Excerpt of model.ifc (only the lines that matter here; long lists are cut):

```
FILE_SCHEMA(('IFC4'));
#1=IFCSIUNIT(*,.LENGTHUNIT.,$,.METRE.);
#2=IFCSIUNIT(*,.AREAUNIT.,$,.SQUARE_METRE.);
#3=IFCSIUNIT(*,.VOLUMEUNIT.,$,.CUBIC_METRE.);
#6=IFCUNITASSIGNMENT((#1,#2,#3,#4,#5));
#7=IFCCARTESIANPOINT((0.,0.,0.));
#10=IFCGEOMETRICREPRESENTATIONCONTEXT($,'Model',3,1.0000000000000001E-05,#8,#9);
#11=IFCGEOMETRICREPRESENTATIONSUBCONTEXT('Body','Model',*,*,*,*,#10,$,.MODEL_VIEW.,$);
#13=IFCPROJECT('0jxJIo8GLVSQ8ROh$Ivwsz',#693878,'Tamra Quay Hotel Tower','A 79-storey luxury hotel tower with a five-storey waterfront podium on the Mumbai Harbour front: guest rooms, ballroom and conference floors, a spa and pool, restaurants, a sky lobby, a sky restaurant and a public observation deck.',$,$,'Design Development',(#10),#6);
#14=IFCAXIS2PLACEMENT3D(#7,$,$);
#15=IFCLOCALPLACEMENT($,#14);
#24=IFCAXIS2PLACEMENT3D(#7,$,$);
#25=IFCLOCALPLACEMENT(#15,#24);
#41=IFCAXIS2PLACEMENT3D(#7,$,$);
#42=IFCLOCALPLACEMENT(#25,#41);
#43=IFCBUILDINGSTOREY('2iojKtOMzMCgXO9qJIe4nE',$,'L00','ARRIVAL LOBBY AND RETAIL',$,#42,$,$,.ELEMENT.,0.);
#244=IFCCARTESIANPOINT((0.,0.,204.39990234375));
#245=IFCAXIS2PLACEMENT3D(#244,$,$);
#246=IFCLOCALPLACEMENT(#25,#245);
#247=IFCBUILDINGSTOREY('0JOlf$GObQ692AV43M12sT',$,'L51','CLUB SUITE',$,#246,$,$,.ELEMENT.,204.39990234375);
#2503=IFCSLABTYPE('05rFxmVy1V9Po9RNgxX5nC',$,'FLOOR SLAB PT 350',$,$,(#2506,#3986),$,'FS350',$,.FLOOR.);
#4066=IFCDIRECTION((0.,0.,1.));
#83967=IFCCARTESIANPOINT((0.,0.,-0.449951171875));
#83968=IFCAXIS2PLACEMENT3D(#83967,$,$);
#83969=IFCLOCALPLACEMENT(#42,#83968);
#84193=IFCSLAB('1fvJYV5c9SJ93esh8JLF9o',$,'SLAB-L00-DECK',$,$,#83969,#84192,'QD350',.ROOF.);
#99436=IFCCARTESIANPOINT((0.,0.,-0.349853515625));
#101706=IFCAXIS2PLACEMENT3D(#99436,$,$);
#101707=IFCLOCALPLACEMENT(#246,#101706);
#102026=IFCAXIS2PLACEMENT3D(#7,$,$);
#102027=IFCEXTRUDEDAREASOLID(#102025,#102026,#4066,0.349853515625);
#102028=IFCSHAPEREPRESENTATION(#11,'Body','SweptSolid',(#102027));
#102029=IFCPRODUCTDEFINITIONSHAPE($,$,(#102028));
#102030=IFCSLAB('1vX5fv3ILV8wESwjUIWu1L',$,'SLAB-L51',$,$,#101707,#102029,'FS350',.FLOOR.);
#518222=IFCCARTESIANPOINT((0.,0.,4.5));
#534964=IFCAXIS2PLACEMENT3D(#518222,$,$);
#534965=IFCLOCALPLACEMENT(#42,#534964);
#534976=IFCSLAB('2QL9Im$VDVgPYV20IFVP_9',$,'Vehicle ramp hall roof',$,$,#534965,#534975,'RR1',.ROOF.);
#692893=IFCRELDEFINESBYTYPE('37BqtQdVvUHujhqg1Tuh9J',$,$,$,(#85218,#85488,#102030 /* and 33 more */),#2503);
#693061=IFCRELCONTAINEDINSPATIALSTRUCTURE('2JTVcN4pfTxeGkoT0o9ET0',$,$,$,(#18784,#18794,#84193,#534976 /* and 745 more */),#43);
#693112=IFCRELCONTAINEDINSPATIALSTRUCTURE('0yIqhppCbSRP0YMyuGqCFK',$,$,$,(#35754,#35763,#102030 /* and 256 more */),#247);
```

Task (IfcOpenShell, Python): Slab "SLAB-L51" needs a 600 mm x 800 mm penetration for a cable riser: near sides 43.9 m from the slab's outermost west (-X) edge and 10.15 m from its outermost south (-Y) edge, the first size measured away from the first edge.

```python
import numpy as np
import ifcopenshell
import ifcopenshell.api.feature
import ifcopenshell.api.geometry
import ifcopenshell.api.root
import ifcopenshell.geom
import ifcopenshell.util.placement
import ifcopenshell.util.representation
import ifcopenshell.util.shape
import ifcopenshell.util.unit

model = ifcopenshell.open("model.ifc")
unit_scale = ifcopenshell.util.unit.calculate_unit_scale(model)
settings = ifcopenshell.geom.settings()


def volume(element):
    """Net volume in cubic metres, openings subtracted."""
    shape = ifcopenshell.geom.create_shape(settings, element)
    return ifcopenshell.util.shape.get_volume(shape.geometry)


slab = model.by_guid("1vX5fv3ILV8wESwjUIWu1L")
before = volume(slab)

# Extent in the slab's own axes, in metres. The edges named are its -X and -Y sides.
slab_shape = ifcopenshell.geom.create_shape(settings, slab)
vertices = ifcopenshell.util.shape.get_vertices(slab_shape.geometry)
x_min, y_min, bottom = vertices.min(axis=0)
top = vertices[:, 2].max()

opening = ifcopenshell.api.root.create_entity(model, ifc_class="IfcOpeningElement", name="Cable riser opening", predefined_type="OPENING")
context = ifcopenshell.util.representation.get_context(model, "Model", "Body", "MODEL_VIEW")
width, depth = 0.6, 0.8
outline = [(0.0, 0.0), (width, 0.0), (width, depth), (0.0, depth), (0.0, 0.0)]
# Overshoot both faces by 50 mm so the cut is clean.
shape = ifcopenshell.api.geometry.add_slab_representation(
    model, context=context, depth=top - bottom + 0.1, polyline=outline
)
ifcopenshell.api.geometry.assign_representation(model, product=opening, representation=shape)

matrix = ifcopenshell.util.placement.get_local_placement(slab.ObjectPlacement)
matrix[:, 3] = matrix @ np.append(np.array([x_min + 43.9, y_min + 10.15, bottom - 0.05]) / unit_scale, 1.0)
ifcopenshell.api.geometry.edit_object_placement(model, product=opening, matrix=matrix, is_si=False)
ifcopenshell.api.feature.add_feature(model, feature=opening, element=slab)

after = volume(slab)

print(f"slab volume {before:.3f} -> {after:.3f} m3")

model.write("model_updated.ifc")
```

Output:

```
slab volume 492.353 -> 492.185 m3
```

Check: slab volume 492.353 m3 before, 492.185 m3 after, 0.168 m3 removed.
